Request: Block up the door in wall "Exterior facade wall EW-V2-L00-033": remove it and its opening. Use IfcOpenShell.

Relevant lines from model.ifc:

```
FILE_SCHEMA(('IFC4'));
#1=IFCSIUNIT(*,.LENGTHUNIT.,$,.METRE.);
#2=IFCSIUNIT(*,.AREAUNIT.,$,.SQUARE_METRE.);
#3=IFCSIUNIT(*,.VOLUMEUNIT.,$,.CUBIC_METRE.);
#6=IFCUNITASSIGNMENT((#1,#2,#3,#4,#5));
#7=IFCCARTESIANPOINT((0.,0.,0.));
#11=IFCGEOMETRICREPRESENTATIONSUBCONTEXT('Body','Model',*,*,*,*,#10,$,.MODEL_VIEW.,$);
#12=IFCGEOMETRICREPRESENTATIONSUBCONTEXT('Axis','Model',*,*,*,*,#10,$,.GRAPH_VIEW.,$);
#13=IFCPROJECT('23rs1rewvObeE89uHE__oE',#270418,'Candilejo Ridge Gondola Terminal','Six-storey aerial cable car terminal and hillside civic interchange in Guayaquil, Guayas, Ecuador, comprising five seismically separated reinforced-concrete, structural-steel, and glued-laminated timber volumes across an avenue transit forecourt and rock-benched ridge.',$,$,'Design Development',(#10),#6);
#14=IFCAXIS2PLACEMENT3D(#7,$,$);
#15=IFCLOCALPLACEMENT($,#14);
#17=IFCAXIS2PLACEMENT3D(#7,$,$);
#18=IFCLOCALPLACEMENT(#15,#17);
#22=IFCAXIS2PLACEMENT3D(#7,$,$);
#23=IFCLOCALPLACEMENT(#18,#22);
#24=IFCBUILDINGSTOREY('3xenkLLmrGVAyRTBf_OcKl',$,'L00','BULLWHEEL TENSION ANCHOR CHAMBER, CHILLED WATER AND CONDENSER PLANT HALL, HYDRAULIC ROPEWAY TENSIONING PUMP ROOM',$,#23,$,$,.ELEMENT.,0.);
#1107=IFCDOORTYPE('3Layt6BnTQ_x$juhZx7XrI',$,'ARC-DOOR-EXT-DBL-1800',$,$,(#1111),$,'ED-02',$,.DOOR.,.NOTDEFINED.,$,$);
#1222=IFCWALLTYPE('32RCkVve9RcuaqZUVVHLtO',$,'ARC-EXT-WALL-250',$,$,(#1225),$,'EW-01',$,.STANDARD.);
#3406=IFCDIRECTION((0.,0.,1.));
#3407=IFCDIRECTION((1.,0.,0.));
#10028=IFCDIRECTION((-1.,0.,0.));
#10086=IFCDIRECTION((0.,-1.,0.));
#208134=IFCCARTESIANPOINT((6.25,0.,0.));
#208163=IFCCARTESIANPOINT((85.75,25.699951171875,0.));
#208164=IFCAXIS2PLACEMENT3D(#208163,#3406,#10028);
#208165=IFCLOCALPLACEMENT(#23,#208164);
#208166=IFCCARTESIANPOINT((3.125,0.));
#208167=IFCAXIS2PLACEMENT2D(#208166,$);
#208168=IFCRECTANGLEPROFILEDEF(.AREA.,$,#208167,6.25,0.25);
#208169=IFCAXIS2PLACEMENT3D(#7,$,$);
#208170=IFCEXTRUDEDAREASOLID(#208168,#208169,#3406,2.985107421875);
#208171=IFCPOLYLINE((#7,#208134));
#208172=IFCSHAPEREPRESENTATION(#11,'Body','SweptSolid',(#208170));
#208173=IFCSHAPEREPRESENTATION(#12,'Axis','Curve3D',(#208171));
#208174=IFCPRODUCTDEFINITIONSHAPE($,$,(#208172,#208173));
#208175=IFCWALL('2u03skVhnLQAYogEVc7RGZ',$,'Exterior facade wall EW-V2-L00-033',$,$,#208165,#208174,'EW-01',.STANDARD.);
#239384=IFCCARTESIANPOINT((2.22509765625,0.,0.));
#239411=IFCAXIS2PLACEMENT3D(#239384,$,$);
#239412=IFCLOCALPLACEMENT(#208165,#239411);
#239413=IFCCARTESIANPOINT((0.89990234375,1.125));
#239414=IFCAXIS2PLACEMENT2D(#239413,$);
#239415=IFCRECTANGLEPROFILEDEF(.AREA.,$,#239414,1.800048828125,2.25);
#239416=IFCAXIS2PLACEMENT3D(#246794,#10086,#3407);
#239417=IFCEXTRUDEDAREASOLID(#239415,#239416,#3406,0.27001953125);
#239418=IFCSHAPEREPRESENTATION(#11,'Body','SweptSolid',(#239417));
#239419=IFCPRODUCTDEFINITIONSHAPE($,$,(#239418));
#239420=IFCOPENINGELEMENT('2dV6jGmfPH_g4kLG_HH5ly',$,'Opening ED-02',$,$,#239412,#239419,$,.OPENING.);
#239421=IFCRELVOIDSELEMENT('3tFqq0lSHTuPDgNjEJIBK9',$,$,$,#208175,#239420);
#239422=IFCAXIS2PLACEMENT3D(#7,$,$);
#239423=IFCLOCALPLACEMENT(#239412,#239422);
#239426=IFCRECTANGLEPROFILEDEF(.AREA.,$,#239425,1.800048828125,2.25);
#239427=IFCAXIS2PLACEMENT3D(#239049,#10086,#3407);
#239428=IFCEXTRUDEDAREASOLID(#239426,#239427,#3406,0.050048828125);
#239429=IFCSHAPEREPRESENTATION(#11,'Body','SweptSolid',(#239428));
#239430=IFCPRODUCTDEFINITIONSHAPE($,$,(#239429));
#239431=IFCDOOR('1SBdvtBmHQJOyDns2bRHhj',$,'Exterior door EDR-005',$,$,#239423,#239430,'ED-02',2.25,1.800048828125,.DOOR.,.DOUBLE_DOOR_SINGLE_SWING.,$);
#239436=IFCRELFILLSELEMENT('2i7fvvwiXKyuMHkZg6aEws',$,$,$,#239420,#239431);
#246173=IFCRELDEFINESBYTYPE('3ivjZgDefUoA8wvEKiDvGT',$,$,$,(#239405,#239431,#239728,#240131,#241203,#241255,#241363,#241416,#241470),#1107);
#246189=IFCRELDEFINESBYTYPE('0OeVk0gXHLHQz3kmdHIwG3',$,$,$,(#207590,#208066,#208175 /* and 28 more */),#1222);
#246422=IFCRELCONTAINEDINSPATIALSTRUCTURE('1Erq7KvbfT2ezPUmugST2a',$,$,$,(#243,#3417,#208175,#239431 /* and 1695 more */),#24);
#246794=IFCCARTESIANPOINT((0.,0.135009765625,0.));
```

```python
import ifcopenshell
import ifcopenshell.api.feature
import ifcopenshell.api.root
import ifcopenshell.geom
import ifcopenshell.util.shape

model = ifcopenshell.open("model.ifc")
settings = ifcopenshell.geom.settings()


def volume(element):
    """Net volume in cubic metres, openings subtracted."""
    shape = ifcopenshell.geom.create_shape(settings, element)
    return ifcopenshell.util.shape.get_volume(shape.geometry)


door = model.by_guid("1SBdvtBmHQJOyDns2bRHhj")
opening = door.FillsVoids[0].RelatingOpeningElement
wall = opening.VoidsElements[0].RelatingBuildingElement
before = volume(wall)

ifcopenshell.api.root.remove_product(model, product=door)
ifcopenshell.api.feature.remove_feature(model, feature=opening)

after = volume(wall)

print(f"wall volume {before:.3f} -> {after:.3f} m3")

model.write("model_v2.ifc")
```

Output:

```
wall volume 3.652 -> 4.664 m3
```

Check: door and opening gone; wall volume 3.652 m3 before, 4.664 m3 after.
